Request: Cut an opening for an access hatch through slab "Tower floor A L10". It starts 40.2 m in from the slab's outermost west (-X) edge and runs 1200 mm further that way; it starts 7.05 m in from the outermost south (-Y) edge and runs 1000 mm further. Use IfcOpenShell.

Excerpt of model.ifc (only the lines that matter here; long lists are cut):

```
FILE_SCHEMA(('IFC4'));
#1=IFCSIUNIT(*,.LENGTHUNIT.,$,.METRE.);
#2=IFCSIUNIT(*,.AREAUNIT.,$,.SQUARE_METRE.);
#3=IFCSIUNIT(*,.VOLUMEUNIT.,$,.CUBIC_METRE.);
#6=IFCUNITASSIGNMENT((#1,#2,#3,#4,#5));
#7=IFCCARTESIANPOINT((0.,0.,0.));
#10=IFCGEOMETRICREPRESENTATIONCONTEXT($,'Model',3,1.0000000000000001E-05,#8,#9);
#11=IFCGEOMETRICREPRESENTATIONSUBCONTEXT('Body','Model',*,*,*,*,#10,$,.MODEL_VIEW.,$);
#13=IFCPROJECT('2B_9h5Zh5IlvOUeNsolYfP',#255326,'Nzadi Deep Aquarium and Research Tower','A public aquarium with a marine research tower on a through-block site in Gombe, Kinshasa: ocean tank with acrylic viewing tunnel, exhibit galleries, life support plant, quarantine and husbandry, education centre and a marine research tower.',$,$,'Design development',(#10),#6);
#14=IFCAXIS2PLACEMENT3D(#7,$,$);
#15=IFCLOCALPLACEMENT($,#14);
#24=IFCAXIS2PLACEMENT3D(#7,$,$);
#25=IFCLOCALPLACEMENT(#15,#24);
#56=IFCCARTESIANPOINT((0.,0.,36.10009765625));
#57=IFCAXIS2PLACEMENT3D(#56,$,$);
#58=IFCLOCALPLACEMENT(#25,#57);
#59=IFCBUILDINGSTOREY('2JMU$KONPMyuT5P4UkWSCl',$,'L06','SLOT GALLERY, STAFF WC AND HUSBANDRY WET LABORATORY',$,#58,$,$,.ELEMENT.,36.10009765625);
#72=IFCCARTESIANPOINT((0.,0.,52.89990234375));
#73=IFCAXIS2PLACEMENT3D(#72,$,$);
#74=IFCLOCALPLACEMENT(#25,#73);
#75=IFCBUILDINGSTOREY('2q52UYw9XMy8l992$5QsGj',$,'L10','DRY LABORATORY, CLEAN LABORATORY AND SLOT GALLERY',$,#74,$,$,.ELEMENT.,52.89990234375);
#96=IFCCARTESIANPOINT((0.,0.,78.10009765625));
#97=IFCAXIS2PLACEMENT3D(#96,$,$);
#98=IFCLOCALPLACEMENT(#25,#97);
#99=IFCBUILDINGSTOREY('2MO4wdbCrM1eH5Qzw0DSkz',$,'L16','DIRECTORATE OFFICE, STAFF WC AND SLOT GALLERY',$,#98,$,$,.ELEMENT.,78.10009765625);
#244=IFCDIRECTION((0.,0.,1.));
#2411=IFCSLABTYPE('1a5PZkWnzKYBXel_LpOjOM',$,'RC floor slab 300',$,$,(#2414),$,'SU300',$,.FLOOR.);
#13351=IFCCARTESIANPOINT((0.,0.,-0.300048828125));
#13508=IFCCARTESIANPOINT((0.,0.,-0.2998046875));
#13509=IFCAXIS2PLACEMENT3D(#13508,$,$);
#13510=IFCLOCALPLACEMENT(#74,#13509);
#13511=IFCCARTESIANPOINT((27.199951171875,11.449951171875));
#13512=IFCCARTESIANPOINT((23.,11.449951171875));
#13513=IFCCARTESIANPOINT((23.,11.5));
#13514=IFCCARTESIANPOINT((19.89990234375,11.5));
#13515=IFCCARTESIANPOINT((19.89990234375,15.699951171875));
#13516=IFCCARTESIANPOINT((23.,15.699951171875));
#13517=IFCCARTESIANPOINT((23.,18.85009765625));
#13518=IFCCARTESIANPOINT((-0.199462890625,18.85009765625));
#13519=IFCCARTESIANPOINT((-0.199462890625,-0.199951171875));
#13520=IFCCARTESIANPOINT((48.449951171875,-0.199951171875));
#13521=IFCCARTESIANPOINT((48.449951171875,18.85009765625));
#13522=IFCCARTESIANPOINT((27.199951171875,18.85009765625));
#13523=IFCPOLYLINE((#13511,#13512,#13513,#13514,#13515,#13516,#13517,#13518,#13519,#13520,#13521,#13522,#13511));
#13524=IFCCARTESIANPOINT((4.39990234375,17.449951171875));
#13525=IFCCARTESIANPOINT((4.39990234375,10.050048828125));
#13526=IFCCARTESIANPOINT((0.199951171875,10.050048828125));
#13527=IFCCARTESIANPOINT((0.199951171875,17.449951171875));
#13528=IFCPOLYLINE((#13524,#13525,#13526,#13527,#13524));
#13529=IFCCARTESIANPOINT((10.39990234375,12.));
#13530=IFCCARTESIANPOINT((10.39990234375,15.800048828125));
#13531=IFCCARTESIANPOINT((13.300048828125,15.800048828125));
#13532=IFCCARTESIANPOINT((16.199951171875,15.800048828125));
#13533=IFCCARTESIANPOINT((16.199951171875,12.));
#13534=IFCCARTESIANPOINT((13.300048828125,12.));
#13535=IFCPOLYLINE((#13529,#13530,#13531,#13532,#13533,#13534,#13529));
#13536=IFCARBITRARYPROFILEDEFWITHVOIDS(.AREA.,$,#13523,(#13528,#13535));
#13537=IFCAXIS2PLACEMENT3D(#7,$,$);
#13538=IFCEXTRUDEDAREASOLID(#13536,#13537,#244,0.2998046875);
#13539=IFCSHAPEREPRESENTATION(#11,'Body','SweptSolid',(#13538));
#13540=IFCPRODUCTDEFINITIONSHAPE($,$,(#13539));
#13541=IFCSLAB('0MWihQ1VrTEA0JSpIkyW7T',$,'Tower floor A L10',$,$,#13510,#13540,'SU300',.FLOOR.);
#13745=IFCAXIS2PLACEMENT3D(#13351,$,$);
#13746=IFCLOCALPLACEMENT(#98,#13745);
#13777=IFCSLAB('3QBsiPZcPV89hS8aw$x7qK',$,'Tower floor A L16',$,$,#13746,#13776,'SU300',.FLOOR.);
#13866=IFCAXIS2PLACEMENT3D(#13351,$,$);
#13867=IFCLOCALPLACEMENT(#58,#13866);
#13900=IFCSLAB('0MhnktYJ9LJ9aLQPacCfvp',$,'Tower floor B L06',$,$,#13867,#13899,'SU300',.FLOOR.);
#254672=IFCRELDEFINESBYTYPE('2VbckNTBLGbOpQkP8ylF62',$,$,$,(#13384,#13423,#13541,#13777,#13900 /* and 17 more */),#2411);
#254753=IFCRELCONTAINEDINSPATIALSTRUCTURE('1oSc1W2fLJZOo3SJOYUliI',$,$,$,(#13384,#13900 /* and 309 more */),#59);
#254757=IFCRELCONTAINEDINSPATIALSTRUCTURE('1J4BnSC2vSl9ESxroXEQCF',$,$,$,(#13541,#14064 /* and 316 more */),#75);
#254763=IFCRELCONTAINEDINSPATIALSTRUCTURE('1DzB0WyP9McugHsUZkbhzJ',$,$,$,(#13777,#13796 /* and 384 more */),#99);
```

```python
import numpy as np
import ifcopenshell
import ifcopenshell.api.feature
import ifcopenshell.api.geometry
import ifcopenshell.api.root
import ifcopenshell.geom
import ifcopenshell.util.placement
import ifcopenshell.util.representation
import ifcopenshell.util.shape
import ifcopenshell.util.unit

model = ifcopenshell.open("model.ifc")
unit_scale = ifcopenshell.util.unit.calculate_unit_scale(model)
settings = ifcopenshell.geom.settings()


def volume(element):
    """Net volume in cubic metres, openings subtracted."""
    shape = ifcopenshell.geom.create_shape(settings, element)
    return ifcopenshell.util.shape.get_volume(shape.geometry)


slab = model.by_guid("0MWihQ1VrTEA0JSpIkyW7T")
before = volume(slab)

# Extent in the slab's own axes, in metres. The edges named are its -X and -Y sides.
slab_shape = ifcopenshell.geom.create_shape(settings, slab)
vertices = ifcopenshell.util.shape.get_vertices(slab_shape.geometry)
x_min, y_min, bottom = vertices.min(axis=0)
top = vertices[:, 2].max()

opening = ifcopenshell.api.root.create_entity(model, ifc_class="IfcOpeningElement", name="Access hatch opening", predefined_type="OPENING")
context = ifcopenshell.util.representation.get_context(model, "Model", "Body", "MODEL_VIEW")
width, depth = 1.2, 1
outline = [(0.0, 0.0), (width, 0.0), (width, depth), (0.0, depth), (0.0, 0.0)]
# Overshoot both faces by 50 mm so the cut is clean.
shape = ifcopenshell.api.geometry.add_slab_representation(
    model, context=context, depth=top - bottom + 0.1, polyline=outline
)
ifcopenshell.api.geometry.assign_representation(model, product=opening, representation=shape)

matrix = ifcopenshell.util.placement.get_local_placement(slab.ObjectPlacement)
matrix[:, 3] = matrix @ np.append(np.array([x_min + 40.2, y_min + 7.05, bottom - 0.05]) / unit_scale, 1.0)
ifcopenshell.api.geometry.edit_object_placement(model, product=opening, matrix=matrix, is_si=False)
ifcopenshell.api.feature.add_feature(model, feature=opening, element=slab)

after = volume(slab)

print(f"slab volume {before:.3f} -> {after:.3f} m3")

model.write("model_edited.ifc")
```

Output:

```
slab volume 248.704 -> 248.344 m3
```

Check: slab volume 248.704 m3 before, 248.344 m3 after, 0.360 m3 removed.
